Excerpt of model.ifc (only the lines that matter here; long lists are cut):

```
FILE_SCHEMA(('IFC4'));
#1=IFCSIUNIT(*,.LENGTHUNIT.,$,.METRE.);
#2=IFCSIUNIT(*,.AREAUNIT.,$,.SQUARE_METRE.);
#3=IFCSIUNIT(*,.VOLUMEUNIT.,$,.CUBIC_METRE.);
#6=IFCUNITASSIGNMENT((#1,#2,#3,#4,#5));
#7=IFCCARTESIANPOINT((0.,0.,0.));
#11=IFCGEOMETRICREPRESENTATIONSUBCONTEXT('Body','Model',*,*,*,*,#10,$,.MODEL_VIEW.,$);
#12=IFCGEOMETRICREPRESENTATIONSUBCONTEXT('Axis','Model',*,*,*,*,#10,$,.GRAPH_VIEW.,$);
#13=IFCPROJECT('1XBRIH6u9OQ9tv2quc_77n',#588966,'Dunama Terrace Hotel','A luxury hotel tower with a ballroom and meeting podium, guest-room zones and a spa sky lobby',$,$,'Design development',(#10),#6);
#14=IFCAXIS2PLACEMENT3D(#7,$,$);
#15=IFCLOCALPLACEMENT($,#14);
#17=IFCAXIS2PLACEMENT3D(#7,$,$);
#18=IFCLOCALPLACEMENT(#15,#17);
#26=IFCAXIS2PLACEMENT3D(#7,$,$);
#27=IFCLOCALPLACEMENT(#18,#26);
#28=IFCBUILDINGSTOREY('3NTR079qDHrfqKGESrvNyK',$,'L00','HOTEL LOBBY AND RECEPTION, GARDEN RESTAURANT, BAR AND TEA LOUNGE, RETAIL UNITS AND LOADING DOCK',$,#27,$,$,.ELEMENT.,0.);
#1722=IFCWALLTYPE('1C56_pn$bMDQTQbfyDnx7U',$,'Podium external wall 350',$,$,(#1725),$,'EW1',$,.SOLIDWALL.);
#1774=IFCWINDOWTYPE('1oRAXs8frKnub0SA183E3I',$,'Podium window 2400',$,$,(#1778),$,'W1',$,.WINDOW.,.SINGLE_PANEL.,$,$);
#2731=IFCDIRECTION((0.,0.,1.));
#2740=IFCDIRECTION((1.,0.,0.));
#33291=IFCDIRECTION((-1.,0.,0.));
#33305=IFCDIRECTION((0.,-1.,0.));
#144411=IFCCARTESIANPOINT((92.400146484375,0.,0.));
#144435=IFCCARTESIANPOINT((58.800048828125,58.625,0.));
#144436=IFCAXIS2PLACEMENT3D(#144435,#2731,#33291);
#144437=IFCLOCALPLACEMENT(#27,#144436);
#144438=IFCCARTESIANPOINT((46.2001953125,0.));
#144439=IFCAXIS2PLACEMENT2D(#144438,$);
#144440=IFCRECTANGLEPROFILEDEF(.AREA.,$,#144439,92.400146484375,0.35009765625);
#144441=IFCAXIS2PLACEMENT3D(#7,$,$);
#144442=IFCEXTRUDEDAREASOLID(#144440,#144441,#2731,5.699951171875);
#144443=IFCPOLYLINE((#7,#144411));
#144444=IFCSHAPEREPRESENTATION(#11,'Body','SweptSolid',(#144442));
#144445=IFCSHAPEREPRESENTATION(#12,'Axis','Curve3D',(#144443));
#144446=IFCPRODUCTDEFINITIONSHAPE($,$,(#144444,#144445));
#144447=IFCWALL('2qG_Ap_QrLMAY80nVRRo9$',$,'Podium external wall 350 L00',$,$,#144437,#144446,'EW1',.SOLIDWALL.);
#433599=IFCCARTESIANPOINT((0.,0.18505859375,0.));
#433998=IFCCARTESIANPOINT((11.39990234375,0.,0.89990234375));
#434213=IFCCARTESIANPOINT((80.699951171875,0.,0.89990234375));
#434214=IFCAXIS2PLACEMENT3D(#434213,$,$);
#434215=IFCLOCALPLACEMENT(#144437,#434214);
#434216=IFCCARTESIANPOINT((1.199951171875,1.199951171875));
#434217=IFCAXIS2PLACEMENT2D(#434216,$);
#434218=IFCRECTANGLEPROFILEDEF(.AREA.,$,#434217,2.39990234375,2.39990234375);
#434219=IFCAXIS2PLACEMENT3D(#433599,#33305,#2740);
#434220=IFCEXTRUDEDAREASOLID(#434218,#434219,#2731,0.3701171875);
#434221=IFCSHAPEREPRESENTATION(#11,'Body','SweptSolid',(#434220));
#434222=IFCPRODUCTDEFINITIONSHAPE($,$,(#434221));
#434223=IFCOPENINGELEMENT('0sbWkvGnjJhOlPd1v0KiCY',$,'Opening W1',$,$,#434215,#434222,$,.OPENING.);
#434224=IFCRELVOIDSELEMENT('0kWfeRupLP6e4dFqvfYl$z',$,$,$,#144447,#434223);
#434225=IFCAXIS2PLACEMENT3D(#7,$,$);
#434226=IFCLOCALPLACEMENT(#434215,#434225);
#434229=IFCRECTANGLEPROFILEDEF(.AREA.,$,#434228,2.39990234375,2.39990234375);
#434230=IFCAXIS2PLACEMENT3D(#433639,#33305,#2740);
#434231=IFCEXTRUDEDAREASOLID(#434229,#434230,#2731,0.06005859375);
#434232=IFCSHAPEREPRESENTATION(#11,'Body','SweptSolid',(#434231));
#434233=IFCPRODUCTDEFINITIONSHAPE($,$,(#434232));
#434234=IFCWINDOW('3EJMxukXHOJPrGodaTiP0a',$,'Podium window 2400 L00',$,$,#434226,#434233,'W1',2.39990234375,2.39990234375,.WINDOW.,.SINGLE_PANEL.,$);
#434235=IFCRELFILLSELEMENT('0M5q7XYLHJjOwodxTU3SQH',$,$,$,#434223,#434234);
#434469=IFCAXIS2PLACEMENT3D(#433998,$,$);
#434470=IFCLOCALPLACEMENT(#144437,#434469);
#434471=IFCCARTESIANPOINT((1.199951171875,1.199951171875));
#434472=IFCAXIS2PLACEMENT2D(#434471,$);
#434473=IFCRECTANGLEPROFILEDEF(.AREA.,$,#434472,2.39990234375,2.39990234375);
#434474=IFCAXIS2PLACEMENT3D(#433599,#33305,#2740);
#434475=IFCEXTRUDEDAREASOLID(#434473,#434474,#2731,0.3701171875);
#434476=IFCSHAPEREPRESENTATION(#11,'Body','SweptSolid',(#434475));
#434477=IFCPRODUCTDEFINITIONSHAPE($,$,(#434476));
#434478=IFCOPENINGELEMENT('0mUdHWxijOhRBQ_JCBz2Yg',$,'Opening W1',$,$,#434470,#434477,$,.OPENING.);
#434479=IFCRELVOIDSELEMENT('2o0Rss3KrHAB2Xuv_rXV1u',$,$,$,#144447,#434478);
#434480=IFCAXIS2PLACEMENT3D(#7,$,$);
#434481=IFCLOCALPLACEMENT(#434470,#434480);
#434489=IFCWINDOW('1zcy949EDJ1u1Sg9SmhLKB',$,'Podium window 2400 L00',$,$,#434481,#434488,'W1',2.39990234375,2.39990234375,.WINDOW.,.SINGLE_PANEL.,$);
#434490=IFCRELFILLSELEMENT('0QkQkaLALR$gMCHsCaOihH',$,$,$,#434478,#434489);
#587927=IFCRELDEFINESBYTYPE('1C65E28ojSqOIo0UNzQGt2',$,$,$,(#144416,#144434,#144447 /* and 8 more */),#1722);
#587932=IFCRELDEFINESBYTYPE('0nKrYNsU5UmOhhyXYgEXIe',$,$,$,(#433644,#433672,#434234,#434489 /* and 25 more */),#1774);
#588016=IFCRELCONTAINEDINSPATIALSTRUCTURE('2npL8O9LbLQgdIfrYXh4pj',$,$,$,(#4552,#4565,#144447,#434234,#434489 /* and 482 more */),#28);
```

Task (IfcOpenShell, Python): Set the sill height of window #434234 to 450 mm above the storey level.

```python
import numpy as np
import ifcopenshell
import ifcopenshell.api.geometry
import ifcopenshell.geom
import ifcopenshell.util.element
import ifcopenshell.util.placement
import ifcopenshell.util.shape
import ifcopenshell.util.unit

model = ifcopenshell.open("model.ifc")
unit_scale = ifcopenshell.util.unit.calculate_unit_scale(model)

window = model.by_guid("3EJMxukXHOJPrGodaTiP0a")
opening = window.FillsVoids[0].RelatingOpeningElement
storey = ifcopenshell.util.element.get_container(window, ifc_class="IfcBuildingStorey")
level = ifcopenshell.util.placement.get_local_placement(storey.ObjectPlacement)[2, 3]

# The opening's origin need not be at the sill, so measure its lowest point.
shape = ifcopenshell.geom.create_shape(ifcopenshell.geom.settings(), opening)
bottom = ifcopenshell.util.shape.get_shape_bottom_elevation(shape, shape.geometry) / unit_scale
dz = level + 0.45 / unit_scale - bottom

shift = np.array([0.0, 0.0, dz])
# The window is placed relative to its opening, so it follows when the opening moves.
matrix = ifcopenshell.util.placement.get_local_placement(opening.ObjectPlacement)
matrix[:3, 3] += shift
ifcopenshell.api.geometry.edit_object_placement(
    model, product=opening, matrix=matrix, is_si=False, should_transform_children=True
)

print(f"moved by {dz * unit_scale:+.3f} m")

model.write("model_v2.ifc")
```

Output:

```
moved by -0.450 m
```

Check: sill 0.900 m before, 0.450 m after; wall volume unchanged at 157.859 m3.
